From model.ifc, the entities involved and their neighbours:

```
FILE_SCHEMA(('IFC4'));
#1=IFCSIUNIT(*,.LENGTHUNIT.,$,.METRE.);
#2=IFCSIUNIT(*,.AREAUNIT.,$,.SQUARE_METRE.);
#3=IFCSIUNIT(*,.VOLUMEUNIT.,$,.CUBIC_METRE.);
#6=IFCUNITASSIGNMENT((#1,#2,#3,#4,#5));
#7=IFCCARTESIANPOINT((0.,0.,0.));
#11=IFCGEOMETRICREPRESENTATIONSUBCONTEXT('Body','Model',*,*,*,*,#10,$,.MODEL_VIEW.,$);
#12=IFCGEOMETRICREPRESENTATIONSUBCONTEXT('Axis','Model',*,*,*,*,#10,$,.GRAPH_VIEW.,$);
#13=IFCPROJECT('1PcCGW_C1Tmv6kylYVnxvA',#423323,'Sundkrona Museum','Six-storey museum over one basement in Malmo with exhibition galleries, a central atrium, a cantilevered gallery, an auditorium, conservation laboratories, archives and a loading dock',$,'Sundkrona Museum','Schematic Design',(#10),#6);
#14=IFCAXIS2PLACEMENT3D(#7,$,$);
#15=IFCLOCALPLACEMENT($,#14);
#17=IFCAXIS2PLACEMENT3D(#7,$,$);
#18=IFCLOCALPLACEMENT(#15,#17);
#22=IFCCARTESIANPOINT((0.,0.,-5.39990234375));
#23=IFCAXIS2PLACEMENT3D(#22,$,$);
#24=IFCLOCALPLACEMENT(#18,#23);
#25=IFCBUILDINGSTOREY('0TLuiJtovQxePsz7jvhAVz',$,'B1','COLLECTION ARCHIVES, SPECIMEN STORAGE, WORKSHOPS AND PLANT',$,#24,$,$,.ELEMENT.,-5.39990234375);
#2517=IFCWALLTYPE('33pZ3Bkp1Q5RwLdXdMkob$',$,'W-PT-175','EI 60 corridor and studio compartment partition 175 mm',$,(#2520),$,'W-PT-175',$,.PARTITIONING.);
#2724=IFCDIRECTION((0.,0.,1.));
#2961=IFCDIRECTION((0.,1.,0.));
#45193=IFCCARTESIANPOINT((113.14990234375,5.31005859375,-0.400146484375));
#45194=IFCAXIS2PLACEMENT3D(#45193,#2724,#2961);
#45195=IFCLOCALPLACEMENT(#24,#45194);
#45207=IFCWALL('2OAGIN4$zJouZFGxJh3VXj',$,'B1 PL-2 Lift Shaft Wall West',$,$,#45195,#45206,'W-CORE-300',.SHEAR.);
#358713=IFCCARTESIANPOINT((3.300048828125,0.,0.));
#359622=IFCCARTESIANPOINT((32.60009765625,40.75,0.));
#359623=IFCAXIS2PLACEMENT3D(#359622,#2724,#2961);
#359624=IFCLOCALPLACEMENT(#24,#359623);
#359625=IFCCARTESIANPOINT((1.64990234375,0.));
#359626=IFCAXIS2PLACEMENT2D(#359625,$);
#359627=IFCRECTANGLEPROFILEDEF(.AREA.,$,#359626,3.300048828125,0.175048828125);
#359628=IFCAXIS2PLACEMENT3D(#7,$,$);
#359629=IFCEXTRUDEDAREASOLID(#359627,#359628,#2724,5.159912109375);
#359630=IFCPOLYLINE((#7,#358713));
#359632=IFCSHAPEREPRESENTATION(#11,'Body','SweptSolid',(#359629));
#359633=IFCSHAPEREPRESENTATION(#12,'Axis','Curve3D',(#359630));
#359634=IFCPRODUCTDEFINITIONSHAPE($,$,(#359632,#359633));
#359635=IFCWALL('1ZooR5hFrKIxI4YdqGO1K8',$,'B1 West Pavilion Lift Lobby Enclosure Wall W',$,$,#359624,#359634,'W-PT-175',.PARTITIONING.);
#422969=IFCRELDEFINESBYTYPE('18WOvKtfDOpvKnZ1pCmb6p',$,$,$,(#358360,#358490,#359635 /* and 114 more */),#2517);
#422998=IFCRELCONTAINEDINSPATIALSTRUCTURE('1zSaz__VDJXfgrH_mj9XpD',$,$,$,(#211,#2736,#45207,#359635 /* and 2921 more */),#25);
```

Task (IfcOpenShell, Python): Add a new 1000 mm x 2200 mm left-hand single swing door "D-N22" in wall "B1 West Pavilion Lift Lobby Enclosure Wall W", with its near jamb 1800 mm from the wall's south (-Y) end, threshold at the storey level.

```python
import numpy as np
import ifcopenshell
import ifcopenshell.api.feature
import ifcopenshell.api.geometry
import ifcopenshell.api.root
import ifcopenshell.api.spatial
import ifcopenshell.geom
import ifcopenshell.util.element
import ifcopenshell.util.placement
import ifcopenshell.util.representation
import ifcopenshell.util.shape
import ifcopenshell.util.unit

model = ifcopenshell.open("model.ifc")
unit_scale = ifcopenshell.util.unit.calculate_unit_scale(model)
settings = ifcopenshell.geom.settings()


def volume(element):
    """Net volume in cubic metres, openings subtracted."""
    shape = ifcopenshell.geom.create_shape(settings, element)
    return ifcopenshell.util.shape.get_volume(shape.geometry)


wall = model.by_guid("1ZooR5hFrKIxI4YdqGO1K8")
storey = ifcopenshell.util.element.get_container(wall, ifc_class="IfcBuildingStorey")
context = ifcopenshell.util.representation.get_context(model, "Model", "Body", "MODEL_VIEW")
before = volume(wall)

width, height, from_end, sill = 1, 2.2, 1.8, 0.0  # metres

# The wall runs along its own X axis, and the end named is its -X end.
wall_shape = ifcopenshell.geom.create_shape(settings, wall)
x, y, z = ifcopenshell.util.shape.get_vertices(wall_shape.geometry).T
start = x.min() + from_end
face, thickness = float(y.min()), float(y.max() - y.min())
wall_matrix = ifcopenshell.util.placement.get_local_placement(wall.ObjectPlacement)
level = ifcopenshell.util.placement.get_local_placement(storey.ObjectPlacement)[2, 3]


def in_wall(x, y):
    """Placement at x, y metres in the wall's axes, at sill height."""
    matrix = wall_matrix.copy()
    matrix[:, 3] = wall_matrix @ np.array([x / unit_scale, y / unit_scale, 0.0, 1.0])
    matrix[2, 3] = level + sill / unit_scale
    return matrix


# Opening: a box that overshoots both wall faces by 50 mm.
opening = ifcopenshell.api.root.create_entity(model, ifc_class="IfcOpeningElement", predefined_type="OPENING")
box = ifcopenshell.api.geometry.add_wall_representation(
    model, context=context, length=width, height=height, thickness=thickness + 0.1
)
ifcopenshell.api.geometry.assign_representation(model, product=opening, representation=box)
ifcopenshell.api.geometry.edit_object_placement(model, product=opening, matrix=in_wall(start, face - 0.05), is_si=False)
ifcopenshell.api.feature.add_feature(model, feature=opening, element=wall)

door = ifcopenshell.api.root.create_entity(model, ifc_class="IfcDoor", name="D-N22", predefined_type="DOOR")
door.OverallWidth, door.OverallHeight = width / unit_scale, height / unit_scale
door.OperationType = "SINGLE_SWING_LEFT"
body = ifcopenshell.api.geometry.add_door_representation(
    model,
    context=context,
    overall_width=door.OverallWidth,
    overall_height=door.OverallHeight,
    operation_type="SINGLE_SWING_LEFT",
    lining_properties={"LiningDepth": thickness / unit_scale, "ThresholdDepth": thickness / unit_scale},
)
ifcopenshell.api.geometry.assign_representation(model, product=door, representation=body)
ifcopenshell.api.spatial.assign_container(model, products=[door], relating_structure=storey)
ifcopenshell.api.feature.add_filling(model, opening=opening, element=door)

# The lining spans the wall, so the door starts at the wall face.
ifcopenshell.api.geometry.edit_object_placement(model, product=door, matrix=in_wall(start, face), is_si=False)

after = volume(wall)

print(f"wall volume {before:.3f} -> {after:.3f} m3")

model.write("model-out.ifc")
```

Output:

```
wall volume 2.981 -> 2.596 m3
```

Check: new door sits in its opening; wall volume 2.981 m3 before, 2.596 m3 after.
